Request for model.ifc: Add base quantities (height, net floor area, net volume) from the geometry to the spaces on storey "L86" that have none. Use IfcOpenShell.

First a look at what the model holds.

```python
import ifcopenshell
import ifcopenshell.util.element
import ifcopenshell.util.unit

model = ifcopenshell.open("model.ifc")
print(model.schema)
for unit_type in ("LENGTHUNIT", "AREAUNIT", "VOLUMEUNIT"):
    print(unit_type, ifcopenshell.util.unit.calculate_unit_scale(model, unit_type))
storey = next(s for s in model.by_type("IfcBuildingStorey") if s.Name == "L86")
spaces = [e for e in ifcopenshell.util.element.get_decomposition(storey) if e.is_a("IfcSpace")]
for e in sorted(spaces, key=lambda e: e.id()):
    print(e.id(), e.is_a(), e.Name, list(ifcopenshell.util.element.get_psets(e, qtos_only=True)), sep=" | ")
```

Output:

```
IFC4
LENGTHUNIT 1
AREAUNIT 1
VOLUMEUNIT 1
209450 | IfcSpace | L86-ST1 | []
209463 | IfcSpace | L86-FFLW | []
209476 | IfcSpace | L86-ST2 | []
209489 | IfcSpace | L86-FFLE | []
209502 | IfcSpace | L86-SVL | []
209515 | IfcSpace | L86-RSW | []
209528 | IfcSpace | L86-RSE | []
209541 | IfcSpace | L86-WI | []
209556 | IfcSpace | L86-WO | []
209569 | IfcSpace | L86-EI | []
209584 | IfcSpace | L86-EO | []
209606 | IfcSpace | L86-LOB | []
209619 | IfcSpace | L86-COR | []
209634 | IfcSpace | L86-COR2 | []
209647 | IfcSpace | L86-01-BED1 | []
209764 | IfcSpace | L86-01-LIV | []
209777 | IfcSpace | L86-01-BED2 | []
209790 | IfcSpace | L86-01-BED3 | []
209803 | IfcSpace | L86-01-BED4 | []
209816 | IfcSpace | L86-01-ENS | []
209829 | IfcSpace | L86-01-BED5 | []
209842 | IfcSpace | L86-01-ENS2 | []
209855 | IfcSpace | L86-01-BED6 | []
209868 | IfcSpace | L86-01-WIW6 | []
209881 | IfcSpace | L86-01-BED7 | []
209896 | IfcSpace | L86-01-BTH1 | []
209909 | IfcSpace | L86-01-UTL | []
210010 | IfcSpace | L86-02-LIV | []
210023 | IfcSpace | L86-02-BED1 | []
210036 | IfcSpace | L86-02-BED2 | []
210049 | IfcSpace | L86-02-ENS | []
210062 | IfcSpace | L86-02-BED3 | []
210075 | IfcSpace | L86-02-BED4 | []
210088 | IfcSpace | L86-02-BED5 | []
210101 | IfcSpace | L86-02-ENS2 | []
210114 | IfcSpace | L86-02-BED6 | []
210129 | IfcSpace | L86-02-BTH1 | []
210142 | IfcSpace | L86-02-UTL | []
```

```python
import ifcopenshell
import ifcopenshell.api.pset
import ifcopenshell.geom
import ifcopenshell.util.element
import ifcopenshell.util.shape
import ifcopenshell.util.unit

model = ifcopenshell.open("model.ifc")
unit_scale = ifcopenshell.util.unit.calculate_unit_scale(model)
area_scale = ifcopenshell.util.unit.calculate_unit_scale(model, "AREAUNIT")
volume_scale = ifcopenshell.util.unit.calculate_unit_scale(model, "VOLUMEUNIT")
settings = ifcopenshell.geom.settings()

storey = next(s for s in model.by_type("IfcBuildingStorey") if s.Name == "L86")
spaces = [e for e in ifcopenshell.util.element.get_decomposition(storey) if e.is_a("IfcSpace")]

for e in sorted(spaces, key=lambda e: e.id()):
    if ifcopenshell.util.element.get_psets(e, qtos_only=True, should_inherit=False):
        continue
    # Geometry comes back in metres, in the element's own axes.
    shape = ifcopenshell.geom.create_shape(settings, e)
    values = {
        "Height": ifcopenshell.util.shape.get_z(shape.geometry) / unit_scale,
        "NetFloorArea": ifcopenshell.util.shape.get_footprint_area(shape.geometry) / area_scale,
        "NetVolume": ifcopenshell.util.shape.get_volume(shape.geometry) / volume_scale,
    }
    qto = ifcopenshell.api.pset.add_qto(model, product=e, name="Qto_SpaceBaseQuantities")
    ifcopenshell.api.pset.edit_qto(model, qto=qto, properties=values)
    print(e.id(), {k: round(v, 3) for k, v in values.items()})

model.write("model_rev.ifc")
```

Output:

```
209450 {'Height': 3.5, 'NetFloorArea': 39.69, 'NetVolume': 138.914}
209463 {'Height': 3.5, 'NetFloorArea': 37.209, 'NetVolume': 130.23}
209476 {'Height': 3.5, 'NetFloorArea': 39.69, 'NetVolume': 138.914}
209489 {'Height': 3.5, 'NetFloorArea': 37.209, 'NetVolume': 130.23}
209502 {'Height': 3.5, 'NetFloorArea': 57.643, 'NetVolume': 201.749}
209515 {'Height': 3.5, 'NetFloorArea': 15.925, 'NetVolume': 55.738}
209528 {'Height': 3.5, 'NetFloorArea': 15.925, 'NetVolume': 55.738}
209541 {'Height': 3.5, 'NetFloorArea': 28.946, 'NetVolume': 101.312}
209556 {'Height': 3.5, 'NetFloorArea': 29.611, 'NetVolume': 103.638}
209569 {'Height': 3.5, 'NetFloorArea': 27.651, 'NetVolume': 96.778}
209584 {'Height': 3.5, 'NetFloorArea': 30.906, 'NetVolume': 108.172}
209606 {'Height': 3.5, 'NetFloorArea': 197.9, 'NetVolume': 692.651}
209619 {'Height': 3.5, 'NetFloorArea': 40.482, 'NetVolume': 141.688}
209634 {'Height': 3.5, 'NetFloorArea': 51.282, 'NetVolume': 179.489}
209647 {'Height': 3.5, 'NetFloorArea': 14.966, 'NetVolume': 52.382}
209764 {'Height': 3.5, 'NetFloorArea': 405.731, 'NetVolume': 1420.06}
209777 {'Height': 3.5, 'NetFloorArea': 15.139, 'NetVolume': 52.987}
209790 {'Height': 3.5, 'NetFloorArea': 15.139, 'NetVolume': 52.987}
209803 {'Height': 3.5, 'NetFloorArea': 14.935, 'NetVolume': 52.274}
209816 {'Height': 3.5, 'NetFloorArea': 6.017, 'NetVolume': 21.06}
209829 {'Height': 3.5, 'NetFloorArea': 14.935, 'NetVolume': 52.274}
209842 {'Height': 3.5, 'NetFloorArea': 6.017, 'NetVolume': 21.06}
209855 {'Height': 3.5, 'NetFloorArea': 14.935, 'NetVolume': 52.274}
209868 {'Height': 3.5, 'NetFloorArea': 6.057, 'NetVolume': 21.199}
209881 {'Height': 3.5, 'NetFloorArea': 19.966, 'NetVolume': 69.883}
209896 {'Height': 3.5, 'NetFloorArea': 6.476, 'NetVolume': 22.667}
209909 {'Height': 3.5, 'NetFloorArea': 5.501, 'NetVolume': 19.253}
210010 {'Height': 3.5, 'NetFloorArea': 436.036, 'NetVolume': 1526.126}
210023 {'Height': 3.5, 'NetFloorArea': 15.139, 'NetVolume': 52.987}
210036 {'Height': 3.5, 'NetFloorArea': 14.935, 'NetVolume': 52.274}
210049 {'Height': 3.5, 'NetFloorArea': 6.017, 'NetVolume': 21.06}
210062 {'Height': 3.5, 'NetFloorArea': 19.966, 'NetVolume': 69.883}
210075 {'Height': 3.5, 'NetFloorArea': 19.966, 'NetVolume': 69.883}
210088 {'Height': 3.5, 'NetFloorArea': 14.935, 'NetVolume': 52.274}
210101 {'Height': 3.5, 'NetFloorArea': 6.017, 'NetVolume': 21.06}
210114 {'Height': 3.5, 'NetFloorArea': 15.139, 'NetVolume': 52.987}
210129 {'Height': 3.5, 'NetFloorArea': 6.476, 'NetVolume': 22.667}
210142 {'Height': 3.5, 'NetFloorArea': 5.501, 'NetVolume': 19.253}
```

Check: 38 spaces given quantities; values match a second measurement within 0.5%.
